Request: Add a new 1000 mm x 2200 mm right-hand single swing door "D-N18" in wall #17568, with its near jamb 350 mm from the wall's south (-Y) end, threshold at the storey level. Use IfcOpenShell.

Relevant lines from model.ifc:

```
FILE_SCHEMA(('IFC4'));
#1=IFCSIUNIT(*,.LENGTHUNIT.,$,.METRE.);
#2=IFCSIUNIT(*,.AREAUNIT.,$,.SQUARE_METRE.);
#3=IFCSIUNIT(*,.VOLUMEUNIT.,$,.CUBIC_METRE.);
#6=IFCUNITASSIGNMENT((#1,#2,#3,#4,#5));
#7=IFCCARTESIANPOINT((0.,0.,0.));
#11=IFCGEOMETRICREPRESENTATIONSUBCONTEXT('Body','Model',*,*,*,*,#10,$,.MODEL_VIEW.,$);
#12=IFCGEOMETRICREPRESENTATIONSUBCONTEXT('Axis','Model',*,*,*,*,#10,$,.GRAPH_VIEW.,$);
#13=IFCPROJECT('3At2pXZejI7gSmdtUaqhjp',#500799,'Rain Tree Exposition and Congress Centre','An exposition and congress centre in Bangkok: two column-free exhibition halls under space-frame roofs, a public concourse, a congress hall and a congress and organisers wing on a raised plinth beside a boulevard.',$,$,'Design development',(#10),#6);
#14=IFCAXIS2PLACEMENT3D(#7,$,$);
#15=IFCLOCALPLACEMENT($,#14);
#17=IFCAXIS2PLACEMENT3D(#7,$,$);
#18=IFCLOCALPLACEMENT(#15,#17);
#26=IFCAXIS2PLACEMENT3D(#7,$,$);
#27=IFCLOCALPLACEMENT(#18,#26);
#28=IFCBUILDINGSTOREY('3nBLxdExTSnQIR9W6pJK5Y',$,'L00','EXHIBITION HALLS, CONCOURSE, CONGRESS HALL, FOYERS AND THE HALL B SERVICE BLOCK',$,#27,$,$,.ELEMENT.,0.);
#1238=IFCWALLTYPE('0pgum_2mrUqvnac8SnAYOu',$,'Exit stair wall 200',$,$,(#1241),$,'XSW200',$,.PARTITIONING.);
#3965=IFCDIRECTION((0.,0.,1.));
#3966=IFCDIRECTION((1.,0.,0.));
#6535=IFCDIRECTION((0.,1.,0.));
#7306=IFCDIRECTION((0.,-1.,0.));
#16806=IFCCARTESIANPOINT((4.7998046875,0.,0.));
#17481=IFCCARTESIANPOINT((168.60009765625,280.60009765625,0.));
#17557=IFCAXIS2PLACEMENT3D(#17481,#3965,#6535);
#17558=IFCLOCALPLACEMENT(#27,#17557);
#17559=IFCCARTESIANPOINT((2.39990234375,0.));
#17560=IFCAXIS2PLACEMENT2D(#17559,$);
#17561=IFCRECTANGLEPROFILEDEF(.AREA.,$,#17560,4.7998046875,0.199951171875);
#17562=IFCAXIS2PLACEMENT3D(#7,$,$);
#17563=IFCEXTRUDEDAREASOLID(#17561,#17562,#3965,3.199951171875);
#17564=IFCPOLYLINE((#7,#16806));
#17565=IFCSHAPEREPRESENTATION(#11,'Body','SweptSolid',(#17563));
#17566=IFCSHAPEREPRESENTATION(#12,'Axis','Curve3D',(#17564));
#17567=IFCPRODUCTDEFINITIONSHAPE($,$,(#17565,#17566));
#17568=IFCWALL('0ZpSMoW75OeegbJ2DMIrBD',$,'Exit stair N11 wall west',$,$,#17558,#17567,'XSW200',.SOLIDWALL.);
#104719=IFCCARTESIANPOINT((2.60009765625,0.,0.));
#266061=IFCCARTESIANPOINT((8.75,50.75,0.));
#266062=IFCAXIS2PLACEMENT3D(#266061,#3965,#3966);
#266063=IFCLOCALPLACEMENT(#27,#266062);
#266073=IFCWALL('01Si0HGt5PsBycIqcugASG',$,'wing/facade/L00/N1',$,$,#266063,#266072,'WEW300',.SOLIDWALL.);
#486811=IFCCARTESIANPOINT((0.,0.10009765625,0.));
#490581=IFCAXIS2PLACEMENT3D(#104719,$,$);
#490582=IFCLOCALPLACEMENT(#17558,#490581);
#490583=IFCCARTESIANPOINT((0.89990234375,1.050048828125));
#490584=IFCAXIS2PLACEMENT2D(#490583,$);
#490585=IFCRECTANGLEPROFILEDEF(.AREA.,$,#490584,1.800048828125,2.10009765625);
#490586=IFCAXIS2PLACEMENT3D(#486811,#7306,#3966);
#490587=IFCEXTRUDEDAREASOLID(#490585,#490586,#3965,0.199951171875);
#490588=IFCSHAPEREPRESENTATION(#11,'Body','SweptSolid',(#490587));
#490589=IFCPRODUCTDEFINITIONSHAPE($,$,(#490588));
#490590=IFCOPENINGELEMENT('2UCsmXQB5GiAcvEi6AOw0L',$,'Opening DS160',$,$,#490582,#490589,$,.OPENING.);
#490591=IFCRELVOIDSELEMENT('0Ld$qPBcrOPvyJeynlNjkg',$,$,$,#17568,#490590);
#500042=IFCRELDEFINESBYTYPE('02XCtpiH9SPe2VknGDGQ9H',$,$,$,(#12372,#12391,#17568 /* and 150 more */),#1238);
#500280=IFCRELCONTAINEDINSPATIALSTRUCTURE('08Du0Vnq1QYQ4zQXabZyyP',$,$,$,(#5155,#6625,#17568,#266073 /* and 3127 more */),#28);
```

```python
import numpy as np
import ifcopenshell
import ifcopenshell.api.feature
import ifcopenshell.api.geometry
import ifcopenshell.api.root
import ifcopenshell.api.spatial
import ifcopenshell.geom
import ifcopenshell.util.element
import ifcopenshell.util.placement
import ifcopenshell.util.representation
import ifcopenshell.util.shape
import ifcopenshell.util.unit

model = ifcopenshell.open("model.ifc")
unit_scale = ifcopenshell.util.unit.calculate_unit_scale(model)
settings = ifcopenshell.geom.settings()


def volume(element):
    """Net volume in cubic metres, openings subtracted."""
    shape = ifcopenshell.geom.create_shape(settings, element)
    return ifcopenshell.util.shape.get_volume(shape.geometry)


wall = model.by_id(17568)
storey = ifcopenshell.util.element.get_container(wall, ifc_class="IfcBuildingStorey")
context = ifcopenshell.util.representation.get_context(model, "Model", "Body", "MODEL_VIEW")
before = volume(wall)

width, height, from_end, sill = 1, 2.2, 0.35, 0.0  # metres

# The wall runs along its own X axis, and the end named is its -X end.
wall_shape = ifcopenshell.geom.create_shape(settings, wall)
x, y, z = ifcopenshell.util.shape.get_vertices(wall_shape.geometry).T
start = x.min() + from_end
face, thickness = float(y.min()), float(y.max() - y.min())
wall_matrix = ifcopenshell.util.placement.get_local_placement(wall.ObjectPlacement)
level = ifcopenshell.util.placement.get_local_placement(storey.ObjectPlacement)[2, 3]


def in_wall(x, y):
    """Placement at x, y metres in the wall's axes, at sill height."""
    matrix = wall_matrix.copy()
    matrix[:, 3] = wall_matrix @ np.array([x / unit_scale, y / unit_scale, 0.0, 1.0])
    matrix[2, 3] = level + sill / unit_scale
    return matrix


# Opening: a box that overshoots both wall faces by 50 mm.
opening = ifcopenshell.api.root.create_entity(model, ifc_class="IfcOpeningElement", predefined_type="OPENING")
box = ifcopenshell.api.geometry.add_wall_representation(
    model, context=context, length=width, height=height, thickness=thickness + 0.1
)
ifcopenshell.api.geometry.assign_representation(model, product=opening, representation=box)
ifcopenshell.api.geometry.edit_object_placement(model, product=opening, matrix=in_wall(start, face - 0.05), is_si=False)
ifcopenshell.api.feature.add_feature(model, feature=opening, element=wall)

door = ifcopenshell.api.root.create_entity(model, ifc_class="IfcDoor", name="D-N18", predefined_type="DOOR")
door.OverallWidth, door.OverallHeight = width / unit_scale, height / unit_scale
door.OperationType = "SINGLE_SWING_RIGHT"
body = ifcopenshell.api.geometry.add_door_representation(
    model,
    context=context,
    overall_width=door.OverallWidth,
    overall_height=door.OverallHeight,
    operation_type="SINGLE_SWING_RIGHT",
    lining_properties={"LiningDepth": thickness / unit_scale, "ThresholdDepth": thickness / unit_scale},
)
ifcopenshell.api.geometry.assign_representation(model, product=door, representation=body)
ifcopenshell.api.spatial.assign_container(model, products=[door], relating_structure=storey)
ifcopenshell.api.feature.add_filling(model, opening=opening, element=door)

# The lining spans the wall, so the door starts at the wall face.
ifcopenshell.api.geometry.edit_object_placement(model, product=door, matrix=in_wall(start, face), is_si=False)

after = volume(wall)

print(f"wall volume {before:.3f} -> {after:.3f} m3")

model.write("model_updated.ifc")
```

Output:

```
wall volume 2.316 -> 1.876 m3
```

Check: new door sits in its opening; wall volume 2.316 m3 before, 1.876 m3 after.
